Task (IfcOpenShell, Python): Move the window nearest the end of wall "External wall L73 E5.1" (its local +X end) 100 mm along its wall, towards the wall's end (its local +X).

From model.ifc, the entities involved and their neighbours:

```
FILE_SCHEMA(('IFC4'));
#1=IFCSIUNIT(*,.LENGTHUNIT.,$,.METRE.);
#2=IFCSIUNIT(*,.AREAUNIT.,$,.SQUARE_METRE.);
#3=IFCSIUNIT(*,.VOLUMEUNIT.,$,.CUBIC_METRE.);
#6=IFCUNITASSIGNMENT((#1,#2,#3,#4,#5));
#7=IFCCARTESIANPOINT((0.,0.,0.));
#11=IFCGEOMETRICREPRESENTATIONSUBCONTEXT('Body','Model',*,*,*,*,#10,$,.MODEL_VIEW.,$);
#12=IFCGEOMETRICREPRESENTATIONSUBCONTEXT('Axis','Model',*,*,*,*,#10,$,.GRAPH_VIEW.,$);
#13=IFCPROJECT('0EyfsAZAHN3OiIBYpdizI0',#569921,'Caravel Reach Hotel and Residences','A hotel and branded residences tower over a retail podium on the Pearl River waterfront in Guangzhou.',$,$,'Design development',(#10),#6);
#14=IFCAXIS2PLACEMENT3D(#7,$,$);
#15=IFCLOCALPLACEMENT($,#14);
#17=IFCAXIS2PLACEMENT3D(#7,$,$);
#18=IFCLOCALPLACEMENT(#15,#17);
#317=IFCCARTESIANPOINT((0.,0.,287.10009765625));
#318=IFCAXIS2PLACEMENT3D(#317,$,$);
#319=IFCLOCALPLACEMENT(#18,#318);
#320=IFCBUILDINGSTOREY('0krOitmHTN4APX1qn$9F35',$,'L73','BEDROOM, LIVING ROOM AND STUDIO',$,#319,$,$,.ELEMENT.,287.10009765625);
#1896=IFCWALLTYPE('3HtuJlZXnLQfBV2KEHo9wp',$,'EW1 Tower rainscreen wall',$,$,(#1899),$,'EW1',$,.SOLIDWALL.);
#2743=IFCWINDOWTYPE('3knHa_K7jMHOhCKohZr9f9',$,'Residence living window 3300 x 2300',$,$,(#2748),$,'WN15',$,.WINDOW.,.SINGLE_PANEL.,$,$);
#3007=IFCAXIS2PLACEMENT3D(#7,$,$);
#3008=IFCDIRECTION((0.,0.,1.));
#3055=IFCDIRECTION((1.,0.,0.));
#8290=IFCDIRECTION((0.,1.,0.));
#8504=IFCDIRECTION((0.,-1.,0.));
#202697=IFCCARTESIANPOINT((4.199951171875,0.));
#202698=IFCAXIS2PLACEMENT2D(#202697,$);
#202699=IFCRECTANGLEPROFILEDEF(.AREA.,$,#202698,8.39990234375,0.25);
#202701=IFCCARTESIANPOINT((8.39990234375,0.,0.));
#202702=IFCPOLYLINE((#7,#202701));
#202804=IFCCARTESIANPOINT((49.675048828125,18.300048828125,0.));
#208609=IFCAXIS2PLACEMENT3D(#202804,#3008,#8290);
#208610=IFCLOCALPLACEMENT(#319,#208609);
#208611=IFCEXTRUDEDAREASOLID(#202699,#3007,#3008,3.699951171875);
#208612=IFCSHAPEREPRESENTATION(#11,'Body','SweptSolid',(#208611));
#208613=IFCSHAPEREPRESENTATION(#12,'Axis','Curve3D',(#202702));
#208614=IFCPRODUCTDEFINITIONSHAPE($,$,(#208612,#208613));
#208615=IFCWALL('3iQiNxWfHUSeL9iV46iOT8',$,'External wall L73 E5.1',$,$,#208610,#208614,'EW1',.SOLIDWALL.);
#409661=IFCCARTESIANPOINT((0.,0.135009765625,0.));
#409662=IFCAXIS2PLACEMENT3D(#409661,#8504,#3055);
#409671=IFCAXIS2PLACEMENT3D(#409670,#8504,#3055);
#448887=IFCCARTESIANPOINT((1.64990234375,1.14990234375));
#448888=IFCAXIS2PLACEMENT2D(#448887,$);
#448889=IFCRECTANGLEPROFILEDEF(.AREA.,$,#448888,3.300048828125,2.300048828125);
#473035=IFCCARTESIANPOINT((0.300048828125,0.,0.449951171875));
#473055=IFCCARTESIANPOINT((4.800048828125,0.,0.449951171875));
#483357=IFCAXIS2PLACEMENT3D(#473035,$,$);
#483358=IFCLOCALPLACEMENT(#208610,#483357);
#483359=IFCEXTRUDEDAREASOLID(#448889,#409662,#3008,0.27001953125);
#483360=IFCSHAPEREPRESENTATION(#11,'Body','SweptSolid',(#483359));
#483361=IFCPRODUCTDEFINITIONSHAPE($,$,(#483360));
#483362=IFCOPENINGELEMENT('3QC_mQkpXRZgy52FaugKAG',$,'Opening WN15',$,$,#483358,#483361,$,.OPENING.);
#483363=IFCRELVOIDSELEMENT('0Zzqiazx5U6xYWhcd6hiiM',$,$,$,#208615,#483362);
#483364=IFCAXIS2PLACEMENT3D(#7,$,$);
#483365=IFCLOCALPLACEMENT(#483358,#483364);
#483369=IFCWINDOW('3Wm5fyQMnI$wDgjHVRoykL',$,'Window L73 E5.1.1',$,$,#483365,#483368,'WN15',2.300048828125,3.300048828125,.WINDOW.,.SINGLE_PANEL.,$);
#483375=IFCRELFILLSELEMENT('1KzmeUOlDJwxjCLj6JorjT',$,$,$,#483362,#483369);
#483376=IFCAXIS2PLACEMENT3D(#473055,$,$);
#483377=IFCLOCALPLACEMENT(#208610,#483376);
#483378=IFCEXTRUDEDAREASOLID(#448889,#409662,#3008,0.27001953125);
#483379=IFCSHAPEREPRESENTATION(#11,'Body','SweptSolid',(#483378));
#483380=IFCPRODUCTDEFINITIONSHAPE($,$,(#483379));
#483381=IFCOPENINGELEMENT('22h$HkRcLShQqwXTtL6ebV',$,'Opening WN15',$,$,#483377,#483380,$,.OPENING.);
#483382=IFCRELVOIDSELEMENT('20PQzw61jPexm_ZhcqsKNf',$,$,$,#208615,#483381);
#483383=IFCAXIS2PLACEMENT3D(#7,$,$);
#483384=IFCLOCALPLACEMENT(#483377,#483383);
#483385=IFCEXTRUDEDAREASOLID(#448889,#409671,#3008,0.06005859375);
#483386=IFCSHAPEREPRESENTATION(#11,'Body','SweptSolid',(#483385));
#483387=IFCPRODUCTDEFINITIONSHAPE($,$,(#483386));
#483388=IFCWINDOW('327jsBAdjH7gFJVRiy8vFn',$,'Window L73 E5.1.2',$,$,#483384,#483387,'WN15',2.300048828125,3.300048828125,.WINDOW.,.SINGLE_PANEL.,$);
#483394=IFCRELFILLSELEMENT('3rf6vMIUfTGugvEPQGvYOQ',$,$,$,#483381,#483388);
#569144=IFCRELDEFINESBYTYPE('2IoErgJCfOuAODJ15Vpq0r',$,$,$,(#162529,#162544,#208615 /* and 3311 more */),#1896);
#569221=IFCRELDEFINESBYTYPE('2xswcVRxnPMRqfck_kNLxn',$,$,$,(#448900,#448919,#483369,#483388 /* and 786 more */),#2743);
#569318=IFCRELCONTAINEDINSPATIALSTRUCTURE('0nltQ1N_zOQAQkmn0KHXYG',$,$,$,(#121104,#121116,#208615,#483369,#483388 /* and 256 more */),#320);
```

```python
import ifcopenshell
import ifcopenshell.api.geometry
import ifcopenshell.util.placement
import ifcopenshell.util.unit

model = ifcopenshell.open("model.ifc")
unit_scale = ifcopenshell.util.unit.calculate_unit_scale(model)

window = model.by_id(483388)
opening = window.FillsVoids[0].RelatingOpeningElement
wall = opening.VoidsElements[0].RelatingBuildingElement

wall_matrix = ifcopenshell.util.placement.get_local_placement(wall.ObjectPlacement)
shift = wall_matrix[:3, 0] * 0.1 / unit_scale
before = ifcopenshell.util.placement.get_local_placement(window.ObjectPlacement)[:3, 3].copy()

# The window is placed relative to its opening, so it follows when the opening moves.
matrix = ifcopenshell.util.placement.get_local_placement(opening.ObjectPlacement)
matrix[:3, 3] += shift
ifcopenshell.api.geometry.edit_object_placement(
    model, product=opening, matrix=matrix, is_si=False, should_transform_children=True
)

after = ifcopenshell.util.placement.get_local_placement(window.ObjectPlacement)[:3, 3]
print("window moved by", (after - before).round(3) + 0.0)

model.write("model_updated.ifc")
```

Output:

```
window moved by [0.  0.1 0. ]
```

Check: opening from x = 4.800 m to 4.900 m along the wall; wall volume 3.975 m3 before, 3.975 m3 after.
